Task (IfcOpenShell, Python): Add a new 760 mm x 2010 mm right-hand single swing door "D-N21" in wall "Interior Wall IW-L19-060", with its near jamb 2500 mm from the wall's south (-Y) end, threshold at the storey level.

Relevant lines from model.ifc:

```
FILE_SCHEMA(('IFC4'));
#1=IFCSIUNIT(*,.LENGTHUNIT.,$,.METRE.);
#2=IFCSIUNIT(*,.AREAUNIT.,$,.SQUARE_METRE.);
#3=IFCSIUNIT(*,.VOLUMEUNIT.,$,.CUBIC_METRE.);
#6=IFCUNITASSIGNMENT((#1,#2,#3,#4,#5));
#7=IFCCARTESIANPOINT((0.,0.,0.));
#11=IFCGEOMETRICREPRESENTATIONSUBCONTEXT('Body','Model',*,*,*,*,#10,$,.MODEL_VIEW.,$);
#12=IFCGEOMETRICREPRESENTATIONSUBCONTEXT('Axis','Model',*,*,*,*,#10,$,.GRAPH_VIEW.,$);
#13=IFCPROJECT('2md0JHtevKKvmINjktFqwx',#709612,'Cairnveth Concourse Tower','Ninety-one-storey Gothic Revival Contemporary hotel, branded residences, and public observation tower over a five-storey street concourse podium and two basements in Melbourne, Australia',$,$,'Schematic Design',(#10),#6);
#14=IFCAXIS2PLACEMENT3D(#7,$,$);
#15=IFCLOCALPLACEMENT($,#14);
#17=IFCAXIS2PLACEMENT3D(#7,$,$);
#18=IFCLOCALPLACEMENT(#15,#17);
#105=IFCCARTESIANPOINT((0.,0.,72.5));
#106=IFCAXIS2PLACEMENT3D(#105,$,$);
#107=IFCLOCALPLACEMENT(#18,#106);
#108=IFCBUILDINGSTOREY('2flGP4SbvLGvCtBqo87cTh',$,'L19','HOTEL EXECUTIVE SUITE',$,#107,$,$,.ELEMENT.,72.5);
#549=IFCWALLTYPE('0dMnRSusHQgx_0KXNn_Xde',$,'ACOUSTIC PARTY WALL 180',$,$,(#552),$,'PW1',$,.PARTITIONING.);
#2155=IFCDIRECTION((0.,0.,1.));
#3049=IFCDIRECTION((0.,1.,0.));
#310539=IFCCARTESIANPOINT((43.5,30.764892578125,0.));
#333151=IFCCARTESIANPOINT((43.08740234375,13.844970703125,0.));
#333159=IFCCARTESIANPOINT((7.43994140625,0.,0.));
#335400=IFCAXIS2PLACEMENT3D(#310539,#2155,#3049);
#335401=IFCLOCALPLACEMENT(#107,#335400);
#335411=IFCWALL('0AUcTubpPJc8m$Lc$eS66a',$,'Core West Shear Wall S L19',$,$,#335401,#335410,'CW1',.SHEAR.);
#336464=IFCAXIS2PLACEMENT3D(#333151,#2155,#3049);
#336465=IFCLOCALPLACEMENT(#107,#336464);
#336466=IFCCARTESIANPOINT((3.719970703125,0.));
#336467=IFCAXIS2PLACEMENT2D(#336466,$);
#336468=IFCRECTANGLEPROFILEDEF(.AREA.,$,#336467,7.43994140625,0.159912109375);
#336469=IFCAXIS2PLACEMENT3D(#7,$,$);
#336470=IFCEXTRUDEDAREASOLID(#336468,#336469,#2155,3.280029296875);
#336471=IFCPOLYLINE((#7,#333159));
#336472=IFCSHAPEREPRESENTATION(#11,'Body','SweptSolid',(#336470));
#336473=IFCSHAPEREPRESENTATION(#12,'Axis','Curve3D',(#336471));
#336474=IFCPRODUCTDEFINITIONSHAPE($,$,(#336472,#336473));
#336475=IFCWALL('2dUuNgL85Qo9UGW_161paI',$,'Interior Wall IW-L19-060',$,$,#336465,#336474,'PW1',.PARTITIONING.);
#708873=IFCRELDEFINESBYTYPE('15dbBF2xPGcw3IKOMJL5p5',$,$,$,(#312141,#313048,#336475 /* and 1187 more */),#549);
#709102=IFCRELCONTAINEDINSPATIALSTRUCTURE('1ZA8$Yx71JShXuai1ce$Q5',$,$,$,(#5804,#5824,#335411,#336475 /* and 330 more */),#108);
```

```python
import numpy as np
import ifcopenshell
import ifcopenshell.api.feature
import ifcopenshell.api.geometry
import ifcopenshell.api.root
import ifcopenshell.api.spatial
import ifcopenshell.geom
import ifcopenshell.util.element
import ifcopenshell.util.placement
import ifcopenshell.util.representation
import ifcopenshell.util.shape
import ifcopenshell.util.unit

model = ifcopenshell.open("model.ifc")
unit_scale = ifcopenshell.util.unit.calculate_unit_scale(model)
settings = ifcopenshell.geom.settings()


def volume(element):
    """Net volume in cubic metres, openings subtracted."""
    shape = ifcopenshell.geom.create_shape(settings, element)
    return ifcopenshell.util.shape.get_volume(shape.geometry)


wall = model.by_guid("2dUuNgL85Qo9UGW_161paI")
storey = ifcopenshell.util.element.get_container(wall, ifc_class="IfcBuildingStorey")
context = ifcopenshell.util.representation.get_context(model, "Model", "Body", "MODEL_VIEW")
before = volume(wall)

width, height, from_end, sill = 0.76, 2.01, 2.5, 0.0  # metres

# The wall runs along its own X axis, and the end named is its -X end.
wall_shape = ifcopenshell.geom.create_shape(settings, wall)
x, y, z = ifcopenshell.util.shape.get_vertices(wall_shape.geometry).T
start = x.min() + from_end
face, thickness = float(y.min()), float(y.max() - y.min())
wall_matrix = ifcopenshell.util.placement.get_local_placement(wall.ObjectPlacement)
level = ifcopenshell.util.placement.get_local_placement(storey.ObjectPlacement)[2, 3]


def in_wall(x, y):
    """Placement at x, y metres in the wall's axes, at sill height."""
    matrix = wall_matrix.copy()
    matrix[:, 3] = wall_matrix @ np.array([x / unit_scale, y / unit_scale, 0.0, 1.0])
    matrix[2, 3] = level + sill / unit_scale
    return matrix


# Opening: a box that overshoots both wall faces by 50 mm.
opening = ifcopenshell.api.root.create_entity(model, ifc_class="IfcOpeningElement", predefined_type="OPENING")
box = ifcopenshell.api.geometry.add_wall_representation(
    model, context=context, length=width, height=height, thickness=thickness + 0.1
)
ifcopenshell.api.geometry.assign_representation(model, product=opening, representation=box)
ifcopenshell.api.geometry.edit_object_placement(model, product=opening, matrix=in_wall(start, face - 0.05), is_si=False)
ifcopenshell.api.feature.add_feature(model, feature=opening, element=wall)

door = ifcopenshell.api.root.create_entity(model, ifc_class="IfcDoor", name="D-N21", predefined_type="DOOR")
door.OverallWidth, door.OverallHeight = width / unit_scale, height / unit_scale
door.OperationType = "SINGLE_SWING_RIGHT"
body = ifcopenshell.api.geometry.add_door_representation(
    model,
    context=context,
    overall_width=door.OverallWidth,
    overall_height=door.OverallHeight,
    operation_type="SINGLE_SWING_RIGHT",
    lining_properties={"LiningDepth": thickness / unit_scale, "ThresholdDepth": thickness / unit_scale},
)
ifcopenshell.api.geometry.assign_representation(model, product=door, representation=body)
ifcopenshell.api.spatial.assign_container(model, products=[door], relating_structure=storey)
ifcopenshell.api.feature.add_filling(model, opening=opening, element=door)

# The lining spans the wall, so the door starts at the wall face.
ifcopenshell.api.geometry.edit_object_placement(model, product=door, matrix=in_wall(start, face), is_si=False)

after = volume(wall)

print(f"wall volume {before:.3f} -> {after:.3f} m3")

model.write("model_v2.ifc")
```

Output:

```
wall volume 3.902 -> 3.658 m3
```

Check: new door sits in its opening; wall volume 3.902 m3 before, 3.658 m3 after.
